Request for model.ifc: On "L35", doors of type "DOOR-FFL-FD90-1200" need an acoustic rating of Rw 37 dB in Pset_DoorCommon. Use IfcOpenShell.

First a look at what the model holds.

```python
import ifcopenshell
import ifcopenshell.util.element

model = ifcopenshell.open("model.ifc")
print(model.schema)
storey = next(s for s in model.by_type("IfcBuildingStorey") if s.Name == "L35")
doors = [e for e in ifcopenshell.util.element.get_decomposition(storey) if e.is_a("IfcDoor")]
seen = {}
for e in doors:
    element_type = ifcopenshell.util.element.get_type(e)
    key = (element_type.Name if element_type != e and element_type else None, ifcopenshell.util.element.get_pset(e, "Pset_DoorCommon", "AcousticRating"))
    seen[key] = seen.get(key, 0) + 1
for (name, value), count in sorted(seen.items(), key=str):
    print(count, "x", name, "|", value)
```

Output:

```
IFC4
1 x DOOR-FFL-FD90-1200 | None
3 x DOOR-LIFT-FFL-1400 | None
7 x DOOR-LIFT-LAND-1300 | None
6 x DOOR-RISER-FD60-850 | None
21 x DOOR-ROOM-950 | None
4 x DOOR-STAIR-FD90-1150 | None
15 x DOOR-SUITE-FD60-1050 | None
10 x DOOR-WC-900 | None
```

```python
import ifcopenshell
import ifcopenshell.api.pset
import ifcopenshell.util.element

model = ifcopenshell.open("model.ifc")

storey = next(s for s in model.by_type("IfcBuildingStorey") if s.Name == "L35")
doors = [e for e in ifcopenshell.util.element.get_decomposition(storey) if e.is_a("IfcDoor")]

count = 0
for e in doors:
    element_type = ifcopenshell.util.element.get_type(e)
    if element_type in (None, e) or element_type.Name != "DOOR-FFL-FD90-1200":
        continue
    found = ifcopenshell.util.element.get_pset(e, "Pset_DoorCommon", should_inherit=False)
    if found:
        pset = model.by_id(found["id"])
        if len(ifcopenshell.util.element.get_elements_by_pset(pset)) > 1:
            pset = ifcopenshell.api.pset.unshare_pset(model, products=[e], pset=pset)[0]
    else:
        pset = ifcopenshell.api.pset.add_pset(model, product=e, name="Pset_DoorCommon")
    ifcopenshell.api.pset.edit_pset(model, pset=pset, properties={"AcousticRating": "Rw 37 dB"})
    count += 1

print(count, "doors updated")

model.write("model-out.ifc")
```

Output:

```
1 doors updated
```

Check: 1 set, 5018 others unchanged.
